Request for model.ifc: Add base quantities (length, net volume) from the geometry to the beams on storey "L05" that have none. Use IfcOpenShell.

First a look at what the model holds.

```python
import ifcopenshell
import ifcopenshell.util.element
import ifcopenshell.util.unit

model = ifcopenshell.open("model.ifc")
print(model.schema)
for unit_type in ("LENGTHUNIT", "AREAUNIT", "VOLUMEUNIT"):
    print(unit_type, ifcopenshell.util.unit.calculate_unit_scale(model, unit_type))
storey = next(s for s in model.by_type("IfcBuildingStorey") if s.Name == "L05")
beams = [e for e in ifcopenshell.util.element.get_decomposition(storey) if e.is_a("IfcBeam")]
for e in sorted(beams, key=lambda e: e.id()):
    print(e.id(), e.is_a(), e.Name, list(ifcopenshell.util.element.get_psets(e, qtos_only=True)), sep=" | ")
```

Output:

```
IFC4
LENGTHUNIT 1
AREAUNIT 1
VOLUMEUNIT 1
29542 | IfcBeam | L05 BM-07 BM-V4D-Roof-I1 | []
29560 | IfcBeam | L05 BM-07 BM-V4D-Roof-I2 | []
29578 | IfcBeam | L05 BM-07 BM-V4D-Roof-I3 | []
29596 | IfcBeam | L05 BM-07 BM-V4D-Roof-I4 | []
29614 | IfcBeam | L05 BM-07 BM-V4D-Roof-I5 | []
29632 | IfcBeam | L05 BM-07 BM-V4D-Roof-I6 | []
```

```python
import ifcopenshell
import ifcopenshell.api.pset
import ifcopenshell.geom
import ifcopenshell.util.element
import ifcopenshell.util.shape
import ifcopenshell.util.unit

model = ifcopenshell.open("model.ifc")
unit_scale = ifcopenshell.util.unit.calculate_unit_scale(model)
volume_scale = ifcopenshell.util.unit.calculate_unit_scale(model, "VOLUMEUNIT")
settings = ifcopenshell.geom.settings()

storey = next(s for s in model.by_type("IfcBuildingStorey") if s.Name == "L05")
beams = [e for e in ifcopenshell.util.element.get_decomposition(storey) if e.is_a("IfcBeam")]

for e in sorted(beams, key=lambda e: e.id()):
    if ifcopenshell.util.element.get_psets(e, qtos_only=True, should_inherit=False):
        continue
    # Geometry comes back in metres, in the element's own axes.
    shape = ifcopenshell.geom.create_shape(settings, e)
    values = {
        "Length": ifcopenshell.util.shape.get_max_xyz(shape.geometry) / unit_scale,
        "NetVolume": ifcopenshell.util.shape.get_volume(shape.geometry) / volume_scale,
    }
    qto = ifcopenshell.api.pset.add_qto(model, product=e, name="Qto_BeamBaseQuantities")
    ifcopenshell.api.pset.edit_qto(model, qto=qto, properties=values)
    print(e.id(), {k: round(v, 3) for k, v in values.items()})

model.write("model_updated.ifc")
```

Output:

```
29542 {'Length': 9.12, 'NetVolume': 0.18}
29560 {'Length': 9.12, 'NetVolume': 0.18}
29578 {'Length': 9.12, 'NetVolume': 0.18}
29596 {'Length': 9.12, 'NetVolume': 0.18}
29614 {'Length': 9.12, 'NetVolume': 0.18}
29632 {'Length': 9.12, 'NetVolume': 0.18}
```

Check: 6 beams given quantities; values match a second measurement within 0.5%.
